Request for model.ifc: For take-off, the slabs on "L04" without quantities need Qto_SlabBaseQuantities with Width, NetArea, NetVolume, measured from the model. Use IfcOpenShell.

First a look at what the model holds.

```python
import ifcopenshell
import ifcopenshell.util.element
import ifcopenshell.util.unit

model = ifcopenshell.open("model.ifc")
print(model.schema)
for unit_type in ("LENGTHUNIT", "AREAUNIT", "VOLUMEUNIT"):
    print(unit_type, ifcopenshell.util.unit.calculate_unit_scale(model, unit_type))
storey = next(s for s in model.by_type("IfcBuildingStorey") if s.Name == "L04")
slabs = [e for e in ifcopenshell.util.element.get_decomposition(storey) if e.is_a("IfcSlab")]
for e in sorted(slabs, key=lambda e: e.id()):
    print(e.id(), e.is_a(), e.Name, list(ifcopenshell.util.element.get_psets(e, qtos_only=True)), sep=" | ")
```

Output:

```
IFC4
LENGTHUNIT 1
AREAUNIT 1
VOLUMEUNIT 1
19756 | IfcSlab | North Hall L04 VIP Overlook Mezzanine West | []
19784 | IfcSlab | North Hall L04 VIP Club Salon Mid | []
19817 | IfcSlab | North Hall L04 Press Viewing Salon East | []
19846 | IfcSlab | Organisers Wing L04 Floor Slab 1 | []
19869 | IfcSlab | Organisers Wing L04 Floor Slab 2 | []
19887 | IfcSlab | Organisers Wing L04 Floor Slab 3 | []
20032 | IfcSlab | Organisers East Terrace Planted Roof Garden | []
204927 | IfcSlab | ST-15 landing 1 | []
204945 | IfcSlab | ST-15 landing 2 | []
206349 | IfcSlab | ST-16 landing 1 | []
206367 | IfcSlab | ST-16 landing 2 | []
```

```python
import ifcopenshell
import ifcopenshell.api.pset
import ifcopenshell.geom
import ifcopenshell.util.element
import ifcopenshell.util.shape
import ifcopenshell.util.unit

model = ifcopenshell.open("model.ifc")
unit_scale = ifcopenshell.util.unit.calculate_unit_scale(model)
area_scale = ifcopenshell.util.unit.calculate_unit_scale(model, "AREAUNIT")
volume_scale = ifcopenshell.util.unit.calculate_unit_scale(model, "VOLUMEUNIT")
settings = ifcopenshell.geom.settings()

storey = next(s for s in model.by_type("IfcBuildingStorey") if s.Name == "L04")
slabs = [e for e in ifcopenshell.util.element.get_decomposition(storey) if e.is_a("IfcSlab")]

for e in sorted(slabs, key=lambda e: e.id()):
    if ifcopenshell.util.element.get_psets(e, qtos_only=True, should_inherit=False):
        continue
    # Geometry comes back in metres, in the element's own axes.
    shape = ifcopenshell.geom.create_shape(settings, e)
    values = {
        "Width": ifcopenshell.util.shape.get_z(shape.geometry) / unit_scale,
        "NetArea": ifcopenshell.util.shape.get_footprint_area(shape.geometry) / area_scale,
        "NetVolume": ifcopenshell.util.shape.get_volume(shape.geometry) / volume_scale,
    }
    qto = ifcopenshell.api.pset.add_qto(model, product=e, name="Qto_SlabBaseQuantities")
    ifcopenshell.api.pset.edit_qto(model, qto=qto, properties=values)
    print(e.id(), {k: round(v, 3) for k, v in values.items()})

model.write("model_edited.ifc")
```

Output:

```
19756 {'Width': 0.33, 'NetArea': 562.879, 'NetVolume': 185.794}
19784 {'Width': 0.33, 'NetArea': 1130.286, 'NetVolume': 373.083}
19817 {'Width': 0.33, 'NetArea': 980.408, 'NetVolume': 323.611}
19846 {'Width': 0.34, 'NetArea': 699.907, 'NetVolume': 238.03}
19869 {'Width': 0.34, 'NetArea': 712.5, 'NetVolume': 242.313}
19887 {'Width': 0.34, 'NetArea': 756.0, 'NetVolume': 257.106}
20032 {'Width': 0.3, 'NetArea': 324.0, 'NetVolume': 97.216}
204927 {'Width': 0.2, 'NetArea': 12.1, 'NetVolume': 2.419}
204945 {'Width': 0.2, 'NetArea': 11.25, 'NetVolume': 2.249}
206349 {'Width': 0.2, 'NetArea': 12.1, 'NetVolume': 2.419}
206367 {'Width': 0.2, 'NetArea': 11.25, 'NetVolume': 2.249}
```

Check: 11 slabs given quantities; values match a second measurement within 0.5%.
